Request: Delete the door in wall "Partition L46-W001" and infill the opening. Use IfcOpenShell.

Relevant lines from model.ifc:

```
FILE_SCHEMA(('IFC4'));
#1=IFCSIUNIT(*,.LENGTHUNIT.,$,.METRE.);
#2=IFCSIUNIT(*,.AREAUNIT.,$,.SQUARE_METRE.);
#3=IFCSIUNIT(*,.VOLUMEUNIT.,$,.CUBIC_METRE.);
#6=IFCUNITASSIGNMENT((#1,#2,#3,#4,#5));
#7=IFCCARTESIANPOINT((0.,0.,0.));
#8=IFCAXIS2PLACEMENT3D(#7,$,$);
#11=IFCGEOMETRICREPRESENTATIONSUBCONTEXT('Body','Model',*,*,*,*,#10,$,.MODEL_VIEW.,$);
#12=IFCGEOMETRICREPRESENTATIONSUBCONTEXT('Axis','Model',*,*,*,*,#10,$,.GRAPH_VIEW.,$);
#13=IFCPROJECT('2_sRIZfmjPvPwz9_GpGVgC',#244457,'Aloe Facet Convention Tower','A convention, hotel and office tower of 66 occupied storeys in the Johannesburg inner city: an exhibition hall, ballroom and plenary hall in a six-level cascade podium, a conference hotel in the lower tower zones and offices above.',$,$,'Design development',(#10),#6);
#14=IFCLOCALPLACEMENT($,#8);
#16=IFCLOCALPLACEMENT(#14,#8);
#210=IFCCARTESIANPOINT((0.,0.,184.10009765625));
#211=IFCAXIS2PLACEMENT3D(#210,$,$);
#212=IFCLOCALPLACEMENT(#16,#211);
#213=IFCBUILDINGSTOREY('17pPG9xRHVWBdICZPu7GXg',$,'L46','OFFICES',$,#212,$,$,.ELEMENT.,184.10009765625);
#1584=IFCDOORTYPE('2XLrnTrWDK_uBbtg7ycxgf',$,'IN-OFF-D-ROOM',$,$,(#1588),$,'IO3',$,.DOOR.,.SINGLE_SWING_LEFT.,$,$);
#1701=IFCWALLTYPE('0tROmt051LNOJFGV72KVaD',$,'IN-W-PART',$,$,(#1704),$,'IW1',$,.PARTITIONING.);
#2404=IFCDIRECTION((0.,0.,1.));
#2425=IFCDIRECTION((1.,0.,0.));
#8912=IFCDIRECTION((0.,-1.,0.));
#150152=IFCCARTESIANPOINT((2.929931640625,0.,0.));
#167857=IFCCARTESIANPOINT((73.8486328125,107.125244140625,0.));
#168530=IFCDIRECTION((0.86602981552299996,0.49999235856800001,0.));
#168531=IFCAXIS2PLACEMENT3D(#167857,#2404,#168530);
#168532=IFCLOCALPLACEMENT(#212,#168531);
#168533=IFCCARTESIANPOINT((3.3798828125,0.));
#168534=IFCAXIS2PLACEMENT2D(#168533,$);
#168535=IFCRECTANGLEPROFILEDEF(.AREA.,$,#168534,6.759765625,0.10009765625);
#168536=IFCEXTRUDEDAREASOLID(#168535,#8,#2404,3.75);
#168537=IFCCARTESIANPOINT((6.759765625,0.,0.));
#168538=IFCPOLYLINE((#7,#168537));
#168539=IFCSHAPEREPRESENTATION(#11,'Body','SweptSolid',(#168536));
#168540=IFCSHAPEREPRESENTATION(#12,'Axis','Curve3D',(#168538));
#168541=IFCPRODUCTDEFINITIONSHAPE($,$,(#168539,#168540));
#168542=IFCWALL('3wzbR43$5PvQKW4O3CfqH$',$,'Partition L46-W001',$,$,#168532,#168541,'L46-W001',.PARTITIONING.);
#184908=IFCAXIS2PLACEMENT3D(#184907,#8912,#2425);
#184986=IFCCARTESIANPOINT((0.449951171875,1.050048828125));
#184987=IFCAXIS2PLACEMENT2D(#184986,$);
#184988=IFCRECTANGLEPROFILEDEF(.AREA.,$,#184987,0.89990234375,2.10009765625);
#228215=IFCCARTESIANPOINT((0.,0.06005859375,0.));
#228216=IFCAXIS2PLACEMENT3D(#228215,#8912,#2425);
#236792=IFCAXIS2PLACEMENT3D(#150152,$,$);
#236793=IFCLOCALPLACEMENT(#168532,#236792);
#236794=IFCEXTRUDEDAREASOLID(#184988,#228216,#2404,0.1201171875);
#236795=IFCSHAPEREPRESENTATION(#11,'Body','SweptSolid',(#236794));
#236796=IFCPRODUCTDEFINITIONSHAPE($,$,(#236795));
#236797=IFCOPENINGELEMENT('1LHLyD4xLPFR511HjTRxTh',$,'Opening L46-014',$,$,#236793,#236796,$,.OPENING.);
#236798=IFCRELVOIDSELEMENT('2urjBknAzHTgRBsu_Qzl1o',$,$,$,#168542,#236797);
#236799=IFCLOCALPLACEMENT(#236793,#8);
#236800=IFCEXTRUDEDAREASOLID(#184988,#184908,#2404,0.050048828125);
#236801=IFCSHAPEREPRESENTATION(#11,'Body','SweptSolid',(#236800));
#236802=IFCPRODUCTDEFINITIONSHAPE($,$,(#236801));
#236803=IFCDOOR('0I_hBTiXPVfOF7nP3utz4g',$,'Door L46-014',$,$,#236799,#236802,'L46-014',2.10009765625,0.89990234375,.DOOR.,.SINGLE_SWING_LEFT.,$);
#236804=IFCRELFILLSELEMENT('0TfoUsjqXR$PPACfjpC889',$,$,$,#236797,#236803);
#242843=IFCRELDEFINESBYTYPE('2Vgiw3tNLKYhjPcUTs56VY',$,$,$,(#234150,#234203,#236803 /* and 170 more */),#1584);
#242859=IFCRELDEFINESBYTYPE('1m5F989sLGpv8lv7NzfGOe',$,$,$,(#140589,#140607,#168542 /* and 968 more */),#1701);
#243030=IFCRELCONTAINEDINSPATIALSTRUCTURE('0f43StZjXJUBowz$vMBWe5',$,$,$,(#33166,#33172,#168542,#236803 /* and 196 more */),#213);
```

```python
import ifcopenshell
import ifcopenshell.api.feature
import ifcopenshell.api.root
import ifcopenshell.geom
import ifcopenshell.util.shape

model = ifcopenshell.open("model.ifc")
settings = ifcopenshell.geom.settings()


def volume(element):
    """Net volume in cubic metres, openings subtracted."""
    shape = ifcopenshell.geom.create_shape(settings, element)
    return ifcopenshell.util.shape.get_volume(shape.geometry)


door = model.by_guid("0I_hBTiXPVfOF7nP3utz4g")
opening = door.FillsVoids[0].RelatingOpeningElement
wall = opening.VoidsElements[0].RelatingBuildingElement
before = volume(wall)

ifcopenshell.api.root.remove_product(model, product=door)
ifcopenshell.api.feature.remove_feature(model, feature=opening)

after = volume(wall)

print(f"wall volume {before:.3f} -> {after:.3f} m3")

model.write("model_v2.ifc")
```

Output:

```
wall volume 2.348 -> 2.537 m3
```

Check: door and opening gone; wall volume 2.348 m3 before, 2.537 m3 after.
